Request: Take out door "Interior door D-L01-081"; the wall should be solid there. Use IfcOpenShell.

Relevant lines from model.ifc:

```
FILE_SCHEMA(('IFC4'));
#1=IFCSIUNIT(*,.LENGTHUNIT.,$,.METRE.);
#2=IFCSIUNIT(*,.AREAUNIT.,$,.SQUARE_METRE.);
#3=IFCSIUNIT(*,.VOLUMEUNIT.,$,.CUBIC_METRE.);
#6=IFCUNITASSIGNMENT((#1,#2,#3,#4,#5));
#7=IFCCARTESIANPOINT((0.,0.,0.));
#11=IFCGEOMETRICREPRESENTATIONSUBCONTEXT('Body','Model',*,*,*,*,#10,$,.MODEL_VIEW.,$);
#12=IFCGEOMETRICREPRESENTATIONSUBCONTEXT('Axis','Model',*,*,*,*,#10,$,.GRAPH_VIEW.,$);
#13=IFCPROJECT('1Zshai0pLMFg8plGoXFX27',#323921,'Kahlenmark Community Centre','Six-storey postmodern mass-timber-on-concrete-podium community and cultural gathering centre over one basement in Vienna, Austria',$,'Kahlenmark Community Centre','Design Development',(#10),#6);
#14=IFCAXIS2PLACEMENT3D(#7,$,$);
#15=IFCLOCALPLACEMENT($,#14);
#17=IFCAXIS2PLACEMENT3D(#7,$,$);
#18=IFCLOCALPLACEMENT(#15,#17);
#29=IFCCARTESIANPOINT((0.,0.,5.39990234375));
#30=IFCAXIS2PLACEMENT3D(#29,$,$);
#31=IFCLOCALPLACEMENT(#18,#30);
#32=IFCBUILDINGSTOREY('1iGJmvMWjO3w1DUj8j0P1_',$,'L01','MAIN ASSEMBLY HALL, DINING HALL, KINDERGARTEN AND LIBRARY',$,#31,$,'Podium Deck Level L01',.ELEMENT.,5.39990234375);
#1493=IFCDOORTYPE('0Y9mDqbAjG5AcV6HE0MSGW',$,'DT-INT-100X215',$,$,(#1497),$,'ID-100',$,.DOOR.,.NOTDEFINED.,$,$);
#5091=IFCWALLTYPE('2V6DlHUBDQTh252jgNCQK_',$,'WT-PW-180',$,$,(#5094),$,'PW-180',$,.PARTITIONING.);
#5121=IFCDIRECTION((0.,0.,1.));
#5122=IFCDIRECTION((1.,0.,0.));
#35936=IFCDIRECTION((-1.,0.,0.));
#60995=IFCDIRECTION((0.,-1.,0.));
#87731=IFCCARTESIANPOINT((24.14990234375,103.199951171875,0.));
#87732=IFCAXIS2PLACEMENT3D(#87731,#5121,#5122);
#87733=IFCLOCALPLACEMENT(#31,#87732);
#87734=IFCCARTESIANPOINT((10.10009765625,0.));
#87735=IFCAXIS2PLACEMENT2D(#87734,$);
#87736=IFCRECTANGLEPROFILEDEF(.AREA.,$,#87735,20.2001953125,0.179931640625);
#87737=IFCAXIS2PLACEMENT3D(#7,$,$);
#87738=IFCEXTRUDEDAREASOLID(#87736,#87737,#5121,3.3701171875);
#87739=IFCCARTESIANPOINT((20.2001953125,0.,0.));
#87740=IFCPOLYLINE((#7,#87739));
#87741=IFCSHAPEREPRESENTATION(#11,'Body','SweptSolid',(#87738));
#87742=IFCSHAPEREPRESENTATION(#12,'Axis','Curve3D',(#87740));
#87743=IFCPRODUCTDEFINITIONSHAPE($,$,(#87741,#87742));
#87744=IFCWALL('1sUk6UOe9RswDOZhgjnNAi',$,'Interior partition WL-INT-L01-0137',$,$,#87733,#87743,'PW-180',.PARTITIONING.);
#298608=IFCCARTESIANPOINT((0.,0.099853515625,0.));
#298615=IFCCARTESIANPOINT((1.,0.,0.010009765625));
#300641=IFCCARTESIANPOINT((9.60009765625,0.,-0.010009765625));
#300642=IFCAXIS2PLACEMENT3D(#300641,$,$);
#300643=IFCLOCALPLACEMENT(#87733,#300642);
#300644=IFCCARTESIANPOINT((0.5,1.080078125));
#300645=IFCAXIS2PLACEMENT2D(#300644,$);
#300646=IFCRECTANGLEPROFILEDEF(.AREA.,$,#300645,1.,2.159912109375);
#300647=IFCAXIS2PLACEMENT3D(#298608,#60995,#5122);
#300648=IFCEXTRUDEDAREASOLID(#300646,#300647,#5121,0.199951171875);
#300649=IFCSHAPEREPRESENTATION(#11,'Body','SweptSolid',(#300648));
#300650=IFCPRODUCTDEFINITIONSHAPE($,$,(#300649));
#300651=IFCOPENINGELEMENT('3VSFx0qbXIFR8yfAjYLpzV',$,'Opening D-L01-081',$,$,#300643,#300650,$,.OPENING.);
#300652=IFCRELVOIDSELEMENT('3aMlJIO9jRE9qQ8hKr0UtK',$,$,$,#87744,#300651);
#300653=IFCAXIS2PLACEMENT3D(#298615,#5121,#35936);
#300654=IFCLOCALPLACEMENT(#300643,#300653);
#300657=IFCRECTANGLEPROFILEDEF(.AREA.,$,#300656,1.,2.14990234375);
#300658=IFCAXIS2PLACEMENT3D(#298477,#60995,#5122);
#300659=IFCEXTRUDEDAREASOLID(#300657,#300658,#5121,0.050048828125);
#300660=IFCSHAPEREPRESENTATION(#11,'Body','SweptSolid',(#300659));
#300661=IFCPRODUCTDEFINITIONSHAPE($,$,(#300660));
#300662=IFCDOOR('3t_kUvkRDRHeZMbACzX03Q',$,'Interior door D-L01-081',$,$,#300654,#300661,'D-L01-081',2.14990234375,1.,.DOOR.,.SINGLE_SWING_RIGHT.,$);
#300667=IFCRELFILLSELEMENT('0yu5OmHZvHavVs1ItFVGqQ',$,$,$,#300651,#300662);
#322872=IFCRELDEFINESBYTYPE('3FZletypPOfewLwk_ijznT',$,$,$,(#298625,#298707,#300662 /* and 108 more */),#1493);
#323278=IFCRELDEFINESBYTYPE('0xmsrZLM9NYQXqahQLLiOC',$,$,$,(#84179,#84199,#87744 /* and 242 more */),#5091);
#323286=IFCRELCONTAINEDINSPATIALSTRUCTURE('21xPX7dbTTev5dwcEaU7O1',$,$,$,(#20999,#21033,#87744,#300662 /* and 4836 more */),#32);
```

```python
import ifcopenshell
import ifcopenshell.api.feature
import ifcopenshell.api.root
import ifcopenshell.geom
import ifcopenshell.util.shape

model = ifcopenshell.open("model.ifc")
settings = ifcopenshell.geom.settings()


def volume(element):
    """Net volume in cubic metres, openings subtracted."""
    shape = ifcopenshell.geom.create_shape(settings, element)
    return ifcopenshell.util.shape.get_volume(shape.geometry)


door = model.by_id(300662)
opening = door.FillsVoids[0].RelatingOpeningElement
wall = opening.VoidsElements[0].RelatingBuildingElement
before = volume(wall)

ifcopenshell.api.root.remove_product(model, product=door)
ifcopenshell.api.feature.remove_feature(model, feature=opening)

after = volume(wall)

print(f"wall volume {before:.3f} -> {after:.3f} m3")

model.write("model_rev.ifc")
```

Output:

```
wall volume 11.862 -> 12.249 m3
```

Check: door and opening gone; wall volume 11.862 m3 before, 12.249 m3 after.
